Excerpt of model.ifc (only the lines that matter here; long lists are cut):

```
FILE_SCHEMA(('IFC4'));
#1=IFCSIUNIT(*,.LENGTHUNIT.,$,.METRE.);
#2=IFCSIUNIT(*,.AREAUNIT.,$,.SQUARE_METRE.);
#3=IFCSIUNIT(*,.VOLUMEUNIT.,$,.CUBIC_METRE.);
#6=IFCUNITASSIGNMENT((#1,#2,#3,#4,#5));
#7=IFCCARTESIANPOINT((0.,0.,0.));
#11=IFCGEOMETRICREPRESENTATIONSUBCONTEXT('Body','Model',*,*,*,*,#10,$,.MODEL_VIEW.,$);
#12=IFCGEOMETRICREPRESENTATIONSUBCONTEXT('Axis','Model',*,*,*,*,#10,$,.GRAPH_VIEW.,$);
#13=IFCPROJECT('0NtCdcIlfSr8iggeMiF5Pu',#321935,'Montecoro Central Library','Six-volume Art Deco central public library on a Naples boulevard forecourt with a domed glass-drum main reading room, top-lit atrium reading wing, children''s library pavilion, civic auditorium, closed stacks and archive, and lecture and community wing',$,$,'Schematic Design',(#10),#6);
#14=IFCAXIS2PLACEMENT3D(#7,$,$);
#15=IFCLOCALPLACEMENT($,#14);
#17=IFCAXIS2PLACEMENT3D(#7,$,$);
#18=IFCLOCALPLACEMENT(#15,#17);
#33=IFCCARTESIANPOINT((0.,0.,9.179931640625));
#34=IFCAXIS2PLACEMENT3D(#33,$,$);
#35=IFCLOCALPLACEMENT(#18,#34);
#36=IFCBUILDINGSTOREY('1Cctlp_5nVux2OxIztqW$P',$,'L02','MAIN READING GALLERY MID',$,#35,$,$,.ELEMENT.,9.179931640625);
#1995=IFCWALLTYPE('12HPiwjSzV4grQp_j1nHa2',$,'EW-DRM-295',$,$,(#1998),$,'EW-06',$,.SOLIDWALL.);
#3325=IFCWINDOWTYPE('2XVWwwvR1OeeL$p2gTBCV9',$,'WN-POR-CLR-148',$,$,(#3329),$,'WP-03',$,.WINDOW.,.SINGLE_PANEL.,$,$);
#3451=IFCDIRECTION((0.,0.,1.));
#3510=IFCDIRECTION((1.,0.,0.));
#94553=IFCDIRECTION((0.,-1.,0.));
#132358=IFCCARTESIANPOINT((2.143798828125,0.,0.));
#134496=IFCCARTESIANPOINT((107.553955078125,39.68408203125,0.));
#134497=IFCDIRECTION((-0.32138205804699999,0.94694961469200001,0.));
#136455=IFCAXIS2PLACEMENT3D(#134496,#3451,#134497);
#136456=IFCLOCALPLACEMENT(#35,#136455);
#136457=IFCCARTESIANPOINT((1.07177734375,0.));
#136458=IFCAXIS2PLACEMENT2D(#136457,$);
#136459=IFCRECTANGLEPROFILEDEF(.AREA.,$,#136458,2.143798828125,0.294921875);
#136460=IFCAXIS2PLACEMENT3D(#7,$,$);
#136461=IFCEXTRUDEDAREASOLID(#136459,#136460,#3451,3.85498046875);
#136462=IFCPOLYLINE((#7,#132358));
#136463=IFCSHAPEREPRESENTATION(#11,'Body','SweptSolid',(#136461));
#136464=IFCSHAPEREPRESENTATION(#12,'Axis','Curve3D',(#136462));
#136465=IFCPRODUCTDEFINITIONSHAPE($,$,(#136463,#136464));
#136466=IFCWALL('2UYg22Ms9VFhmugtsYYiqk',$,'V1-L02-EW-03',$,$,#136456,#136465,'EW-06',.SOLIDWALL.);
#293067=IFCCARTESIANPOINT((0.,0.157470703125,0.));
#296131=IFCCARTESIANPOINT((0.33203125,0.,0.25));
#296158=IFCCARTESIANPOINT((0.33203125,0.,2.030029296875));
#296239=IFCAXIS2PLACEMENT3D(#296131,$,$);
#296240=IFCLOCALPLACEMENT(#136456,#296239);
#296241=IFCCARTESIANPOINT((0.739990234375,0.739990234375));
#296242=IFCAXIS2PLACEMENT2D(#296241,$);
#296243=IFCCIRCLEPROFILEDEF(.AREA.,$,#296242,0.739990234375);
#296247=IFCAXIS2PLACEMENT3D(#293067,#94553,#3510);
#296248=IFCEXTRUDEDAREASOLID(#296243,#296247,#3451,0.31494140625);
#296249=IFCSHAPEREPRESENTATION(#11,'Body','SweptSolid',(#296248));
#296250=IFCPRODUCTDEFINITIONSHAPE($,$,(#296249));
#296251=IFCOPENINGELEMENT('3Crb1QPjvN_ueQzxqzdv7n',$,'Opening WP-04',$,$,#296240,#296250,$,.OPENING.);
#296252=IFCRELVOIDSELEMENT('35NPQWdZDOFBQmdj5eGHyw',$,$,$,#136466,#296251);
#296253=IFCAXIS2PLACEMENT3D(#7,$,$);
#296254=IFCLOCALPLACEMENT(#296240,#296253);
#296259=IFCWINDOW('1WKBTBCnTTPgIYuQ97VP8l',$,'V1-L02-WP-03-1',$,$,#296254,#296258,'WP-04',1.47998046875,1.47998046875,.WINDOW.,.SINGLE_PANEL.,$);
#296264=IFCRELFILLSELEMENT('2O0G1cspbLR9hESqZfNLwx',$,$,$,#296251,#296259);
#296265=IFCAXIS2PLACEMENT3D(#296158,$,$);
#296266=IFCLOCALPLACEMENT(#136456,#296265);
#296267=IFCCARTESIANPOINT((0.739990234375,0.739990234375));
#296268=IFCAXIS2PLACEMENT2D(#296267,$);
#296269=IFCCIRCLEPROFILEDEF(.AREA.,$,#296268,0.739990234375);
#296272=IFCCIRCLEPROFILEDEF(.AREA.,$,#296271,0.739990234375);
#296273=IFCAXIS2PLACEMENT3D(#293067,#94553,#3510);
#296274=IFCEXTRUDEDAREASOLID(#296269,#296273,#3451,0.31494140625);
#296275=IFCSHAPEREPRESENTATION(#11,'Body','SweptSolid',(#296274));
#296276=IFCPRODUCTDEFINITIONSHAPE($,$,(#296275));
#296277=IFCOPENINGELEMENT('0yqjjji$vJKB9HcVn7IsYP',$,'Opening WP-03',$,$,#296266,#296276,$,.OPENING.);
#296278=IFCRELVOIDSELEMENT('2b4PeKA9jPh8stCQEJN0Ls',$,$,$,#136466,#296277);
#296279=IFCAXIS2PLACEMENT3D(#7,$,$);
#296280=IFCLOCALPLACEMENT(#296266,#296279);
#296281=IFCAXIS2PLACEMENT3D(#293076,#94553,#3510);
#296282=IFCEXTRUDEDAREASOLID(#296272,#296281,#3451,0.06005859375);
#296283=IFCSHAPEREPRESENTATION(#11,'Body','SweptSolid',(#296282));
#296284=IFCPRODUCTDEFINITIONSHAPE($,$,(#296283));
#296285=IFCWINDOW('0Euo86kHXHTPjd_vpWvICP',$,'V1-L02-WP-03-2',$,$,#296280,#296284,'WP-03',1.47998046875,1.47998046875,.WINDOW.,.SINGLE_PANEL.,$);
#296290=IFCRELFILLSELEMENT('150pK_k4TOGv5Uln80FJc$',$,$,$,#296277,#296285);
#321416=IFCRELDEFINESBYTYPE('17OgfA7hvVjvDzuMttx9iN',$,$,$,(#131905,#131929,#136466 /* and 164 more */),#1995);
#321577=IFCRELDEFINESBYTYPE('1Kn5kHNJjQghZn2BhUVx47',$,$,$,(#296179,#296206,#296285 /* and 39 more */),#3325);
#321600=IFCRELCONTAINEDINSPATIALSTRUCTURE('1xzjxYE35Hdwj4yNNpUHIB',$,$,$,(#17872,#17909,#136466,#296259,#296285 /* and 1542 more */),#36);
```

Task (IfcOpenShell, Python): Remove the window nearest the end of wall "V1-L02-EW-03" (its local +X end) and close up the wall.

```python
import ifcopenshell
import ifcopenshell.api.feature
import ifcopenshell.api.root
import ifcopenshell.geom
import ifcopenshell.util.shape

model = ifcopenshell.open("model.ifc")
settings = ifcopenshell.geom.settings()


def volume(element):
    """Net volume in cubic metres, openings subtracted."""
    shape = ifcopenshell.geom.create_shape(settings, element)
    return ifcopenshell.util.shape.get_volume(shape.geometry)


window = model.by_guid("0Euo86kHXHTPjd_vpWvICP")
opening = window.FillsVoids[0].RelatingOpeningElement
wall = opening.VoidsElements[0].RelatingBuildingElement
before = volume(wall)

ifcopenshell.api.root.remove_product(model, product=window)
ifcopenshell.api.feature.remove_feature(model, feature=opening)

after = volume(wall)

print(f"wall volume {before:.3f} -> {after:.3f} m3")

model.write("model_edited.ifc")
```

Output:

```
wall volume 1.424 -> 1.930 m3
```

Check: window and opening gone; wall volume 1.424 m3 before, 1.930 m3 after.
